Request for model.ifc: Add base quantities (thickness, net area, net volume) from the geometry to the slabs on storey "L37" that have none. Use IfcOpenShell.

First a look at what the model holds.

```python
import ifcopenshell
import ifcopenshell.util.element
import ifcopenshell.util.unit

model = ifcopenshell.open("model.ifc")
print(model.schema)
for unit_type in ("LENGTHUNIT", "AREAUNIT", "VOLUMEUNIT"):
    print(unit_type, ifcopenshell.util.unit.calculate_unit_scale(model, unit_type))
storey = next(s for s in model.by_type("IfcBuildingStorey") if s.Name == "L37")
slabs = [e for e in ifcopenshell.util.element.get_decomposition(storey) if e.is_a("IfcSlab")]
for e in sorted(slabs, key=lambda e: e.id()):
    print(e.id(), e.is_a(), e.Name, list(ifcopenshell.util.element.get_psets(e, qtos_only=True)), sep=" | ")
```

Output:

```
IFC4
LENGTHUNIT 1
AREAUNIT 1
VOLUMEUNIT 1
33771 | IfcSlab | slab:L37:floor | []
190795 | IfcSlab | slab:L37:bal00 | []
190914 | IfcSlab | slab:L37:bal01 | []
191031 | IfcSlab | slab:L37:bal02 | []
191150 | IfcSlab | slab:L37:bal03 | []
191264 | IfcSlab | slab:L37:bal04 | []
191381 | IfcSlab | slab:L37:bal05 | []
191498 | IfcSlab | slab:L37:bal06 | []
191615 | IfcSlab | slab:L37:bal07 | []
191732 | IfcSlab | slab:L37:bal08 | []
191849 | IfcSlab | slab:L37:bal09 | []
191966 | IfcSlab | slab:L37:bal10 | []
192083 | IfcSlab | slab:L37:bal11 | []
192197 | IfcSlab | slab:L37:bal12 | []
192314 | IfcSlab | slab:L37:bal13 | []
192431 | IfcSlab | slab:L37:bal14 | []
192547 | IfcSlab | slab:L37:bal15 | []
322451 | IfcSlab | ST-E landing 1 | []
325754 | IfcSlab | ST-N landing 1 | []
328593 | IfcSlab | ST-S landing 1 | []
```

```python
import ifcopenshell
import ifcopenshell.api.pset
import ifcopenshell.geom
import ifcopenshell.util.element
import ifcopenshell.util.shape
import ifcopenshell.util.unit

model = ifcopenshell.open("model.ifc")
unit_scale = ifcopenshell.util.unit.calculate_unit_scale(model)
area_scale = ifcopenshell.util.unit.calculate_unit_scale(model, "AREAUNIT")
volume_scale = ifcopenshell.util.unit.calculate_unit_scale(model, "VOLUMEUNIT")
settings = ifcopenshell.geom.settings()

storey = next(s for s in model.by_type("IfcBuildingStorey") if s.Name == "L37")
slabs = [e for e in ifcopenshell.util.element.get_decomposition(storey) if e.is_a("IfcSlab")]

for e in sorted(slabs, key=lambda e: e.id()):
    if ifcopenshell.util.element.get_psets(e, qtos_only=True, should_inherit=False):
        continue
    # Geometry comes back in metres, in the element's own axes.
    shape = ifcopenshell.geom.create_shape(settings, e)
    values = {
        "Width": ifcopenshell.util.shape.get_z(shape.geometry) / unit_scale,
        "NetArea": ifcopenshell.util.shape.get_footprint_area(shape.geometry) / area_scale,
        "NetVolume": ifcopenshell.util.shape.get_volume(shape.geometry) / volume_scale,
    }
    qto = ifcopenshell.api.pset.add_qto(model, product=e, name="Qto_SlabBaseQuantities")
    ifcopenshell.api.pset.edit_qto(model, qto=qto, properties=values)
    print(e.id(), {k: round(v, 3) for k, v in values.items()})

model.write("model-out.ifc")
```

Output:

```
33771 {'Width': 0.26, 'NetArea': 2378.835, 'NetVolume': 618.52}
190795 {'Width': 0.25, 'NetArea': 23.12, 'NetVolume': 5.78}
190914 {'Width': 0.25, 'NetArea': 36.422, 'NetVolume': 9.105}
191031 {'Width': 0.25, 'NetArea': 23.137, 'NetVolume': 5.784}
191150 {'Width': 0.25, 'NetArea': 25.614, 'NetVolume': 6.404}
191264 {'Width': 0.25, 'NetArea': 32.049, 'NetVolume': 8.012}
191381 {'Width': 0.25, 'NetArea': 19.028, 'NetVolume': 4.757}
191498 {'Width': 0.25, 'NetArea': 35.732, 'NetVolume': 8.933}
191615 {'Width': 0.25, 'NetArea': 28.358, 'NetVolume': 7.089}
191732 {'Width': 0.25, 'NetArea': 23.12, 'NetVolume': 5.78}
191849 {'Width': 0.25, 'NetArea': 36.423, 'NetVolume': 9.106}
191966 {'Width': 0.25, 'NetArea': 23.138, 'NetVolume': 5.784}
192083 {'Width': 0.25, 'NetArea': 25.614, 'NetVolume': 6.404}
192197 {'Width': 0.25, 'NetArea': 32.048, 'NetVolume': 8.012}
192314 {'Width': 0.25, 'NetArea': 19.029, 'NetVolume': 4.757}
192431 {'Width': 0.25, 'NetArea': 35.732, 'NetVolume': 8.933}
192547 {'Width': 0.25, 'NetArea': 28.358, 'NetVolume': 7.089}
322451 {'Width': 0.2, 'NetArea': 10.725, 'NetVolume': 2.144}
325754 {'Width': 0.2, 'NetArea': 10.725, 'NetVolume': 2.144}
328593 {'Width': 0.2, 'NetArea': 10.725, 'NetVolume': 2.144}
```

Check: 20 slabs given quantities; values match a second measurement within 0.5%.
